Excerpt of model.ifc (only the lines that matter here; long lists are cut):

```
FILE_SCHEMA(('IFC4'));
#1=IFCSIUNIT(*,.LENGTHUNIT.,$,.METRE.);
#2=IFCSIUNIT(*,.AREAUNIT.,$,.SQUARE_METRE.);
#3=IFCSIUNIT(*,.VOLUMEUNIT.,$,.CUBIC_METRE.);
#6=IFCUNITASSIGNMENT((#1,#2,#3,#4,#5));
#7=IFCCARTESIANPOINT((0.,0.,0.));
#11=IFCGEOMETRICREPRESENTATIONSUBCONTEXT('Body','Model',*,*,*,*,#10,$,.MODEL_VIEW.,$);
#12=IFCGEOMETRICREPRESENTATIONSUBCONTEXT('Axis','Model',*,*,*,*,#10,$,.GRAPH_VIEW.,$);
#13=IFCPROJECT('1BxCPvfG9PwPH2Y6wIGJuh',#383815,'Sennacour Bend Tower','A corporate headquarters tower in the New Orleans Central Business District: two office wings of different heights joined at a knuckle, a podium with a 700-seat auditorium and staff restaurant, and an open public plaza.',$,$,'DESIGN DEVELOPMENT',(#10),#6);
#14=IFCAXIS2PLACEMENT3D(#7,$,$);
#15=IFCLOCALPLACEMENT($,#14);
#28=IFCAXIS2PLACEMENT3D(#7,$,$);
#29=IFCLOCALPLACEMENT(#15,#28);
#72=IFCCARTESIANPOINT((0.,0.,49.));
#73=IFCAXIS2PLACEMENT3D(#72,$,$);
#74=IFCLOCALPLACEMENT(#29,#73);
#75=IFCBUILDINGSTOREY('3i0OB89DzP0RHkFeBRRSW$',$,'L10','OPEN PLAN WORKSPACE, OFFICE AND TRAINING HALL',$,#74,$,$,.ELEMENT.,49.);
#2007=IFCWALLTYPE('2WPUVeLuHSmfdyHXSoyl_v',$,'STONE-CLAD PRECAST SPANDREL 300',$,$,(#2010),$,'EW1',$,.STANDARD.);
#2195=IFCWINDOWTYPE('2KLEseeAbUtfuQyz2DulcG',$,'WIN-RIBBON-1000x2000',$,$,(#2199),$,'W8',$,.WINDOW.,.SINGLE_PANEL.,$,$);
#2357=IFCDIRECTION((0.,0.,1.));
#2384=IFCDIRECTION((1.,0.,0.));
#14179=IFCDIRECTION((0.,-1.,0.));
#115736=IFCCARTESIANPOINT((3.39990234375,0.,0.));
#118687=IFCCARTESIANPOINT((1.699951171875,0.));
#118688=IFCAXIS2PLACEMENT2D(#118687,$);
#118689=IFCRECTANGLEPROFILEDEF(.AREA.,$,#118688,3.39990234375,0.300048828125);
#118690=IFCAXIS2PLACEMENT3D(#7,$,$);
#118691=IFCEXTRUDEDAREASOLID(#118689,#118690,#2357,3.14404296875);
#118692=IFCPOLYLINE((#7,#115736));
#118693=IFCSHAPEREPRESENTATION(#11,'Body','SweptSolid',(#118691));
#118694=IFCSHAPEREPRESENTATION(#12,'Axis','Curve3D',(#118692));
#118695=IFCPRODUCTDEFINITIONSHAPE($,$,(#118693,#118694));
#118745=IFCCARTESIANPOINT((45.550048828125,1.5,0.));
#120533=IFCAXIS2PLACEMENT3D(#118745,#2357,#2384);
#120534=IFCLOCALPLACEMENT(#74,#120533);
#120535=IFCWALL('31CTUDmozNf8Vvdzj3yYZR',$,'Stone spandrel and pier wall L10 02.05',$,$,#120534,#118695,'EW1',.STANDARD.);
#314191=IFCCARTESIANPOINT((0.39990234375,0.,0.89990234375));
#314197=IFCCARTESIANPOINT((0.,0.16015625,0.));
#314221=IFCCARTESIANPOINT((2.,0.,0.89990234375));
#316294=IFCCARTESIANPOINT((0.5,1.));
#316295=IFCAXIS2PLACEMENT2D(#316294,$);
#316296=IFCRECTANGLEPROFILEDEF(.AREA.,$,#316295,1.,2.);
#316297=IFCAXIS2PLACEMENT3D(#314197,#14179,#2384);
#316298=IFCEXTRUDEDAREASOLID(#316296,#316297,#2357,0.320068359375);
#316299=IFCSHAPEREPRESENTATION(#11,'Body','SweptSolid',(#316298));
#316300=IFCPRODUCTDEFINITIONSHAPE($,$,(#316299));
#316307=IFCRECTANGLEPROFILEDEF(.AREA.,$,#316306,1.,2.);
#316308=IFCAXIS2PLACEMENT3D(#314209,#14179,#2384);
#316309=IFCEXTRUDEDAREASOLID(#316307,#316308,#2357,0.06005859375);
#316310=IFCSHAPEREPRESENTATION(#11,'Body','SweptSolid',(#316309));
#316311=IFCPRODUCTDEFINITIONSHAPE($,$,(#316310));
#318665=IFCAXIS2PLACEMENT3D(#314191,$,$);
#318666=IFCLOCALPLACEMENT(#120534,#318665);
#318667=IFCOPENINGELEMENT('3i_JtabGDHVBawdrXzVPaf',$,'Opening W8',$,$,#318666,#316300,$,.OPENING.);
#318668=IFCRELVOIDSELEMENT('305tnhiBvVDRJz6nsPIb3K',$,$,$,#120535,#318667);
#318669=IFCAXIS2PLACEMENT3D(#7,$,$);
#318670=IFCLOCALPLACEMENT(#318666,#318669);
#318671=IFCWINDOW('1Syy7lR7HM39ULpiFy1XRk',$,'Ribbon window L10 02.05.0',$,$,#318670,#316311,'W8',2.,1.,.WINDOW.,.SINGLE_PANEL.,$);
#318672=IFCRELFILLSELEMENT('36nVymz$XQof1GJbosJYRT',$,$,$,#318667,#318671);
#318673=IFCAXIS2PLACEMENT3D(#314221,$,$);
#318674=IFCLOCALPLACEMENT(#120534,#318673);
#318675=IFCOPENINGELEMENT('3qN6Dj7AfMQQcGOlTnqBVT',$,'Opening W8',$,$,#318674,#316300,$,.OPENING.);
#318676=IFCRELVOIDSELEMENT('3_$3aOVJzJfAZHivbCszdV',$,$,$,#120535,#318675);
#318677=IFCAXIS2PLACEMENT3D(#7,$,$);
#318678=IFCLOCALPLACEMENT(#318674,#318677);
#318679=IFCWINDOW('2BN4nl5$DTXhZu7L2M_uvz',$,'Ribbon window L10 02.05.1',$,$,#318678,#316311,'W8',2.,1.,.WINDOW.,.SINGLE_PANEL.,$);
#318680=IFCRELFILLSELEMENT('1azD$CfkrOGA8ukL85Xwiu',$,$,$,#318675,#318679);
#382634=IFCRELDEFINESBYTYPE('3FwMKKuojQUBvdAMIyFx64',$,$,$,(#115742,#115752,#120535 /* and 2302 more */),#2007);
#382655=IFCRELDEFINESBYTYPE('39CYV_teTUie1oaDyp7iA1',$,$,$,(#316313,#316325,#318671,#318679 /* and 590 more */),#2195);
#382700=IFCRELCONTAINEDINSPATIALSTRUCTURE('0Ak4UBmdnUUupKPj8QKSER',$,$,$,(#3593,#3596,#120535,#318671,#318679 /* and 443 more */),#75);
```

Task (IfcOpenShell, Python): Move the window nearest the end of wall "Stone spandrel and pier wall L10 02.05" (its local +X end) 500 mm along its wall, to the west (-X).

```python
import ifcopenshell
import ifcopenshell.api.geometry
import ifcopenshell.util.placement
import ifcopenshell.util.unit

model = ifcopenshell.open("model.ifc")
unit_scale = ifcopenshell.util.unit.calculate_unit_scale(model)

window = model.by_guid("2BN4nl5$DTXhZu7L2M_uvz")
opening = window.FillsVoids[0].RelatingOpeningElement
wall = opening.VoidsElements[0].RelatingBuildingElement

wall_matrix = ifcopenshell.util.placement.get_local_placement(wall.ObjectPlacement)
shift = wall_matrix[:3, 0] * -0.5 / unit_scale
before = ifcopenshell.util.placement.get_local_placement(window.ObjectPlacement)[:3, 3].copy()

# The window is placed relative to its opening, so it follows when the opening moves.
matrix = ifcopenshell.util.placement.get_local_placement(opening.ObjectPlacement)
matrix[:3, 3] += shift
ifcopenshell.api.geometry.edit_object_placement(
    model, product=opening, matrix=matrix, is_si=False, should_transform_children=True
)

after = ifcopenshell.util.placement.get_local_placement(window.ObjectPlacement)[:3, 3]
print("window moved by", (after - before).round(3) + 0.0)

model.write("model_edited.ifc")
```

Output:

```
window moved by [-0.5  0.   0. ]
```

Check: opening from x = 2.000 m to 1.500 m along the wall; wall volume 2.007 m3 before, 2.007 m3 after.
